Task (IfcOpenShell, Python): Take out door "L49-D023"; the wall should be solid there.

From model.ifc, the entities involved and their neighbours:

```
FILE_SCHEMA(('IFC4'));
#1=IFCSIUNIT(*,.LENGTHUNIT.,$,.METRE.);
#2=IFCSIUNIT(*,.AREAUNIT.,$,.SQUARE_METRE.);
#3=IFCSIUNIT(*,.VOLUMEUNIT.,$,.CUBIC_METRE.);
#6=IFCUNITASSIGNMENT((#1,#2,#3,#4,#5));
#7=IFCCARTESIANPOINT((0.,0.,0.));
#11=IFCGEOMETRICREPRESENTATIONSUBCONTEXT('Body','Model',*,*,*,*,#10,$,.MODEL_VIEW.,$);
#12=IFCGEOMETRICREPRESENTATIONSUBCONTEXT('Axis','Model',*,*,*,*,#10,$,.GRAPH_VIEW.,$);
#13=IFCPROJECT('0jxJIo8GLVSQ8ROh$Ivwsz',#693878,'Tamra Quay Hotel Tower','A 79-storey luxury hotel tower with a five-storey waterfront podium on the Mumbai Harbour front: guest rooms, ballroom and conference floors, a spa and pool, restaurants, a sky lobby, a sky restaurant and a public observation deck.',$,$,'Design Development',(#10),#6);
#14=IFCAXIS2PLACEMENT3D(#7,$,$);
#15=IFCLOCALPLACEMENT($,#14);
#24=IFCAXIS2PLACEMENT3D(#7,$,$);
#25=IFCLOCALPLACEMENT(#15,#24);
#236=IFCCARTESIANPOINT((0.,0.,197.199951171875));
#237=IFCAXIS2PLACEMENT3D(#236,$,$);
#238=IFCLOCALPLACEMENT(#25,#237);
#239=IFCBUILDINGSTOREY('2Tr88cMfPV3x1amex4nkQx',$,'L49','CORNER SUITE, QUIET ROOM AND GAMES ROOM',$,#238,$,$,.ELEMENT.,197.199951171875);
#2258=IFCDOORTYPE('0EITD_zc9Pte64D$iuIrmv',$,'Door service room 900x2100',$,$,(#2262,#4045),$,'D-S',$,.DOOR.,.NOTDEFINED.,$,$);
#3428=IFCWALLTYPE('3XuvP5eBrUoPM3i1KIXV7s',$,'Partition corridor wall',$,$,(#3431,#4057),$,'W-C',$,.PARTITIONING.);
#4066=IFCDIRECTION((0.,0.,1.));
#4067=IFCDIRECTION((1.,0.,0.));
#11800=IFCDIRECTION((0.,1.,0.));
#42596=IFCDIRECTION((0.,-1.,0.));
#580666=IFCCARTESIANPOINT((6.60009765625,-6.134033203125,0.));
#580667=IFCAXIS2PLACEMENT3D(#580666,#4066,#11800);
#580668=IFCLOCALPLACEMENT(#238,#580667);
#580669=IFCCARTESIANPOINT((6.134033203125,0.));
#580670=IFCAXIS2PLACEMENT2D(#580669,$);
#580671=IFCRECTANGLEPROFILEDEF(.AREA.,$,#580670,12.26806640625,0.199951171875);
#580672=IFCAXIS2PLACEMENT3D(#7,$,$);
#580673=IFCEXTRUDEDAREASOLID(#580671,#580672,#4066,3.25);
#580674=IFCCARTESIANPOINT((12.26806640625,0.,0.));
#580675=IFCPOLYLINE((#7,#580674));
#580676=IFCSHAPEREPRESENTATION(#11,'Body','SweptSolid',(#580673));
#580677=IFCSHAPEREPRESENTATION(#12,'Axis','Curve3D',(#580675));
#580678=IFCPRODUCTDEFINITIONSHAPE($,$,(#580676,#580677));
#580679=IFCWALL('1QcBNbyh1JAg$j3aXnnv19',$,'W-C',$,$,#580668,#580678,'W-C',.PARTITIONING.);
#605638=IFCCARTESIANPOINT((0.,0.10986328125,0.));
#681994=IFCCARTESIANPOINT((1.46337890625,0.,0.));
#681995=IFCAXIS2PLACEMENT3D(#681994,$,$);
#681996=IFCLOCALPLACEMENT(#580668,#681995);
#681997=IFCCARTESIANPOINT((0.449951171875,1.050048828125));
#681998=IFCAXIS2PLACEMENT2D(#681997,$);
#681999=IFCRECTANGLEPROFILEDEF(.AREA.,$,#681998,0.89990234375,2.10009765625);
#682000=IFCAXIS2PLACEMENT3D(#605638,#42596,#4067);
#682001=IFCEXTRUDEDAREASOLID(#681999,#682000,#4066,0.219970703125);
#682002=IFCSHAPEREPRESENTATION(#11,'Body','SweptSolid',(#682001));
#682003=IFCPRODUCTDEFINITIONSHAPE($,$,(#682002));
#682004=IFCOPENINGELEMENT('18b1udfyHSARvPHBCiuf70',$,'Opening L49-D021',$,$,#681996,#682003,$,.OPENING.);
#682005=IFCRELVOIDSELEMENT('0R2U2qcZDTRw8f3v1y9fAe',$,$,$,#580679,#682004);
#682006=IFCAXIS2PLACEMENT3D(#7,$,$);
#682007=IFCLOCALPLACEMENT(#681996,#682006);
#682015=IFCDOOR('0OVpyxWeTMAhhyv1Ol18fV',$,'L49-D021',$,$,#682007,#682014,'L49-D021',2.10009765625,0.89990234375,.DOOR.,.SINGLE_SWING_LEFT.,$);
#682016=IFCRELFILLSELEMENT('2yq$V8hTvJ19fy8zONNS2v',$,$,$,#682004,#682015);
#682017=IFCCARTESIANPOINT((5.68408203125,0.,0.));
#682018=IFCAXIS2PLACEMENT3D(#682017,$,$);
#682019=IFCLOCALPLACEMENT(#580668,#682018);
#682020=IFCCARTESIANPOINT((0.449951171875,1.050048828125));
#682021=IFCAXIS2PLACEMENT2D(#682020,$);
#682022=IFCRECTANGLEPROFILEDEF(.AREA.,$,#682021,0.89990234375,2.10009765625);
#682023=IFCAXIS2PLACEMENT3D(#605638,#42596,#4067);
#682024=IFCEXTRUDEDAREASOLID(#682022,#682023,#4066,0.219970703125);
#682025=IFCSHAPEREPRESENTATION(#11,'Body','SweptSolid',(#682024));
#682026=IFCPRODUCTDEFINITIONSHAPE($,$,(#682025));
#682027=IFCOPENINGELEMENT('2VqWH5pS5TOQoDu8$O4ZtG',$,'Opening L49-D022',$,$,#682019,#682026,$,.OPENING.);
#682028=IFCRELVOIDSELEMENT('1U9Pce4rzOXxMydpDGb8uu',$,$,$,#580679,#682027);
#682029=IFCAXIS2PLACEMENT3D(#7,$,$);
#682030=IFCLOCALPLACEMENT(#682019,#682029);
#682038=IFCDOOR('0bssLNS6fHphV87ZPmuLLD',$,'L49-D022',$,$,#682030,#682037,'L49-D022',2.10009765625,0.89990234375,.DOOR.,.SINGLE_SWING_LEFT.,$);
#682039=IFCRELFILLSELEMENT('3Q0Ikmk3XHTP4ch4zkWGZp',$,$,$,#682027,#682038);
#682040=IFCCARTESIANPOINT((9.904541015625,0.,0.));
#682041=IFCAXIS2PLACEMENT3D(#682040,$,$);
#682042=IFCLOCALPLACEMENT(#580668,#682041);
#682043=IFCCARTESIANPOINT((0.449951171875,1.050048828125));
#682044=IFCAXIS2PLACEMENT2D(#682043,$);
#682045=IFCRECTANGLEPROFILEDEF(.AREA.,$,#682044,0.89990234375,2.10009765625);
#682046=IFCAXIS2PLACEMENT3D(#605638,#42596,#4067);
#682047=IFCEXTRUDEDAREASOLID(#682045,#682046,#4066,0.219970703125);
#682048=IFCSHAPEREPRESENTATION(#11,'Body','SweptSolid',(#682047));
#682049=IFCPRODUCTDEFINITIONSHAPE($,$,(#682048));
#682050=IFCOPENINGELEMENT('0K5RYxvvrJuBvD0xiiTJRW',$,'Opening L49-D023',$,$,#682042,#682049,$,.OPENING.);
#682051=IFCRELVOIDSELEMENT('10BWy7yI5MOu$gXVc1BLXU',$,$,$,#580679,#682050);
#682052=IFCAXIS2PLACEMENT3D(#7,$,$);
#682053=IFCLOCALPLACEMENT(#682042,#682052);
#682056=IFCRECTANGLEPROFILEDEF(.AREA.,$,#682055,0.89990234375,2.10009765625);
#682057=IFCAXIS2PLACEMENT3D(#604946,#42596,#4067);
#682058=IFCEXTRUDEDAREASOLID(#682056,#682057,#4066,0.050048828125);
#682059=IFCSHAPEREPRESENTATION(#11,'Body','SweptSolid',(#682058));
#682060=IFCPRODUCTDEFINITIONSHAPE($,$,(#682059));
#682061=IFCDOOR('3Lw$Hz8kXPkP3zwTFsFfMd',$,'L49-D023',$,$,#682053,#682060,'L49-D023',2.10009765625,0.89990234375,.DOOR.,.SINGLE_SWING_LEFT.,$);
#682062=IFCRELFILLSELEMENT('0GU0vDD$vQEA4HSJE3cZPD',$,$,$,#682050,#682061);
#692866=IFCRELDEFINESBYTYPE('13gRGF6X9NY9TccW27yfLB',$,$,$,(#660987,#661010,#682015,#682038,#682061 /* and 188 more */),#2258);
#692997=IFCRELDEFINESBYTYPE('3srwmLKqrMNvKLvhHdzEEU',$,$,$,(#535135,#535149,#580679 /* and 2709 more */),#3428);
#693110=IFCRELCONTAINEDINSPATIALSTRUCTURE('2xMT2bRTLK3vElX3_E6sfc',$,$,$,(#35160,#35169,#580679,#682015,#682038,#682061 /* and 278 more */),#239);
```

```python
import ifcopenshell
import ifcopenshell.api.feature
import ifcopenshell.api.root
import ifcopenshell.geom
import ifcopenshell.util.shape

model = ifcopenshell.open("model.ifc")
settings = ifcopenshell.geom.settings()


def volume(element):
    """Net volume in cubic metres, openings subtracted."""
    shape = ifcopenshell.geom.create_shape(settings, element)
    return ifcopenshell.util.shape.get_volume(shape.geometry)


door = model.by_guid("3Lw$Hz8kXPkP3zwTFsFfMd")
opening = door.FillsVoids[0].RelatingOpeningElement
wall = opening.VoidsElements[0].RelatingBuildingElement
before = volume(wall)

ifcopenshell.api.root.remove_product(model, product=door)
ifcopenshell.api.feature.remove_feature(model, feature=opening)

after = volume(wall)

print(f"wall volume {before:.3f} -> {after:.3f} m3")

model.write("model_rev.ifc")
```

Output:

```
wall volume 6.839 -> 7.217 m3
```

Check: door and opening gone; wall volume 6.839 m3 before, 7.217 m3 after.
